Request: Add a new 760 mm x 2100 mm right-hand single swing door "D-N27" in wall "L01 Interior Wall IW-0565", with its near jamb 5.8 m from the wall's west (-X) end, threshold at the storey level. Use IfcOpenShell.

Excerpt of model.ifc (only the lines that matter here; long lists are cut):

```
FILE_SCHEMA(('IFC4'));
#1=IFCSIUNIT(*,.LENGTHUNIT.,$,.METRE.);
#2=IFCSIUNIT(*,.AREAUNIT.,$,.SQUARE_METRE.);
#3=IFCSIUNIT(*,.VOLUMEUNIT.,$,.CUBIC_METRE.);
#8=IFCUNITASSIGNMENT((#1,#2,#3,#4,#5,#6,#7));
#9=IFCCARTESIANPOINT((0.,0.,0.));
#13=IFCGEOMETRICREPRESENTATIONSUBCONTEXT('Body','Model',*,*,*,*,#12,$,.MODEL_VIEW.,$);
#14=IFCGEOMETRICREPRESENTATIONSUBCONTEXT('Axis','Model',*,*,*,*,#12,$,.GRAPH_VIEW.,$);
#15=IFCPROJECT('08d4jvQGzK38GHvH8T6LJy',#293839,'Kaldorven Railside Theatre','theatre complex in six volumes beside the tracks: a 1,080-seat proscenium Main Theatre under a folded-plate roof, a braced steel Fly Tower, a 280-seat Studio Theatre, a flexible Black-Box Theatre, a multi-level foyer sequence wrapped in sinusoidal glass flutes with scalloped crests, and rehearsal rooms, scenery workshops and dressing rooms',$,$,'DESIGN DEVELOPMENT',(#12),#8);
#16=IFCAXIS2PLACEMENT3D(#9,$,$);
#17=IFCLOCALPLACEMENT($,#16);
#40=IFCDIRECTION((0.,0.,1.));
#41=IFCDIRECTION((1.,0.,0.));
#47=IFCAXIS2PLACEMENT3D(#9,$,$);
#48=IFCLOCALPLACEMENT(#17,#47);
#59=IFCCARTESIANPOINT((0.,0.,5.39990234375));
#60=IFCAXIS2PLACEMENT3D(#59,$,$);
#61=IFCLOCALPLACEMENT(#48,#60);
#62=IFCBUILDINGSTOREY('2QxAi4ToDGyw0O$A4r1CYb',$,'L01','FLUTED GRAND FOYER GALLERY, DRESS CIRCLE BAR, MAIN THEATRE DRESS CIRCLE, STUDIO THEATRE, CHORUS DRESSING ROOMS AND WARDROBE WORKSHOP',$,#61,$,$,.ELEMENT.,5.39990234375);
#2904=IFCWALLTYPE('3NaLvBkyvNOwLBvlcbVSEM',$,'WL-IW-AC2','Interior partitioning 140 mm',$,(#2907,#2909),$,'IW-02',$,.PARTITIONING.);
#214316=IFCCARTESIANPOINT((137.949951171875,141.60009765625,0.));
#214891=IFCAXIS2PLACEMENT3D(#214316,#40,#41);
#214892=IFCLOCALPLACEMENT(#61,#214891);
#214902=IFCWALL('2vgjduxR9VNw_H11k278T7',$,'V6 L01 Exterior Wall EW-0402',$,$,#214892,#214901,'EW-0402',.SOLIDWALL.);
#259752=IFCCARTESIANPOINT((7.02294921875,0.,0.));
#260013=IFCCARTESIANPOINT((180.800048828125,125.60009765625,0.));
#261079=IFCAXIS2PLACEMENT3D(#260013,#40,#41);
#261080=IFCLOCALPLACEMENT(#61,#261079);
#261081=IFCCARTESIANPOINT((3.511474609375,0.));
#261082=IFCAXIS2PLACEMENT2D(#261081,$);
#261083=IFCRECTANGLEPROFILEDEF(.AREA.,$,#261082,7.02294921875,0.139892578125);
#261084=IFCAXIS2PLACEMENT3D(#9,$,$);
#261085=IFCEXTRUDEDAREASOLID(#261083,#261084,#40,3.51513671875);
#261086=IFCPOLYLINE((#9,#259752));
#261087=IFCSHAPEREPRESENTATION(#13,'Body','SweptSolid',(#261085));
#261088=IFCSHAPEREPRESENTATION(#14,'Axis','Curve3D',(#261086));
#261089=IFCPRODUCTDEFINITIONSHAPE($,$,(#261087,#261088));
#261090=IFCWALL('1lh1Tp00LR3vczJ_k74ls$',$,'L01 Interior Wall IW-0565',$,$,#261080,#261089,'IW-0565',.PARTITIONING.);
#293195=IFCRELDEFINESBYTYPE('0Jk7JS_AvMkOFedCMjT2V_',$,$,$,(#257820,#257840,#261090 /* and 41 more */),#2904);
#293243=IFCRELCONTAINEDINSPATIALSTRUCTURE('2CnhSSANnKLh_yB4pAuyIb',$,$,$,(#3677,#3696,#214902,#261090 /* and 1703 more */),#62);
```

```python
import numpy as np
import ifcopenshell
import ifcopenshell.api.feature
import ifcopenshell.api.geometry
import ifcopenshell.api.root
import ifcopenshell.api.spatial
import ifcopenshell.geom
import ifcopenshell.util.element
import ifcopenshell.util.placement
import ifcopenshell.util.representation
import ifcopenshell.util.shape
import ifcopenshell.util.unit

model = ifcopenshell.open("model.ifc")
unit_scale = ifcopenshell.util.unit.calculate_unit_scale(model)
settings = ifcopenshell.geom.settings()


def volume(element):
    """Net volume in cubic metres, openings subtracted."""
    shape = ifcopenshell.geom.create_shape(settings, element)
    return ifcopenshell.util.shape.get_volume(shape.geometry)


wall = model.by_guid("1lh1Tp00LR3vczJ_k74ls$")
storey = ifcopenshell.util.element.get_container(wall, ifc_class="IfcBuildingStorey")
context = ifcopenshell.util.representation.get_context(model, "Model", "Body", "MODEL_VIEW")
before = volume(wall)

width, height, from_end, sill = 0.76, 2.1, 5.8, 0.0  # metres

# The wall runs along its own X axis, and the end named is its -X end.
wall_shape = ifcopenshell.geom.create_shape(settings, wall)
x, y, z = ifcopenshell.util.shape.get_vertices(wall_shape.geometry).T
start = x.min() + from_end
face, thickness = float(y.min()), float(y.max() - y.min())
wall_matrix = ifcopenshell.util.placement.get_local_placement(wall.ObjectPlacement)
level = ifcopenshell.util.placement.get_local_placement(storey.ObjectPlacement)[2, 3]


def in_wall(x, y):
    """Placement at x, y metres in the wall's axes, at sill height."""
    matrix = wall_matrix.copy()
    matrix[:, 3] = wall_matrix @ np.array([x / unit_scale, y / unit_scale, 0.0, 1.0])
    matrix[2, 3] = level + sill / unit_scale
    return matrix


# Opening: a box that overshoots both wall faces by 50 mm.
opening = ifcopenshell.api.root.create_entity(model, ifc_class="IfcOpeningElement", predefined_type="OPENING")
box = ifcopenshell.api.geometry.add_wall_representation(
    model, context=context, length=width, height=height, thickness=thickness + 0.1
)
ifcopenshell.api.geometry.assign_representation(model, product=opening, representation=box)
ifcopenshell.api.geometry.edit_object_placement(model, product=opening, matrix=in_wall(start, face - 0.05), is_si=False)
ifcopenshell.api.feature.add_feature(model, feature=opening, element=wall)

door = ifcopenshell.api.root.create_entity(model, ifc_class="IfcDoor", name="D-N27", predefined_type="DOOR")
door.OverallWidth, door.OverallHeight = width / unit_scale, height / unit_scale
door.OperationType = "SINGLE_SWING_RIGHT"
body = ifcopenshell.api.geometry.add_door_representation(
    model,
    context=context,
    overall_width=door.OverallWidth,
    overall_height=door.OverallHeight,
    operation_type="SINGLE_SWING_RIGHT",
    lining_properties={"LiningDepth": thickness / unit_scale, "ThresholdDepth": thickness / unit_scale},
)
ifcopenshell.api.geometry.assign_representation(model, product=door, representation=body)
ifcopenshell.api.spatial.assign_container(model, products=[door], relating_structure=storey)
ifcopenshell.api.feature.add_filling(model, opening=opening, element=door)

# The lining spans the wall, so the door starts at the wall face.
ifcopenshell.api.geometry.edit_object_placement(model, product=door, matrix=in_wall(start, face), is_si=False)

after = volume(wall)

print(f"wall volume {before:.3f} -> {after:.3f} m3")

model.write("model_rev.ifc")
```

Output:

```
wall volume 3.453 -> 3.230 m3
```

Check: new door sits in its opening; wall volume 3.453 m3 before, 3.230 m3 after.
